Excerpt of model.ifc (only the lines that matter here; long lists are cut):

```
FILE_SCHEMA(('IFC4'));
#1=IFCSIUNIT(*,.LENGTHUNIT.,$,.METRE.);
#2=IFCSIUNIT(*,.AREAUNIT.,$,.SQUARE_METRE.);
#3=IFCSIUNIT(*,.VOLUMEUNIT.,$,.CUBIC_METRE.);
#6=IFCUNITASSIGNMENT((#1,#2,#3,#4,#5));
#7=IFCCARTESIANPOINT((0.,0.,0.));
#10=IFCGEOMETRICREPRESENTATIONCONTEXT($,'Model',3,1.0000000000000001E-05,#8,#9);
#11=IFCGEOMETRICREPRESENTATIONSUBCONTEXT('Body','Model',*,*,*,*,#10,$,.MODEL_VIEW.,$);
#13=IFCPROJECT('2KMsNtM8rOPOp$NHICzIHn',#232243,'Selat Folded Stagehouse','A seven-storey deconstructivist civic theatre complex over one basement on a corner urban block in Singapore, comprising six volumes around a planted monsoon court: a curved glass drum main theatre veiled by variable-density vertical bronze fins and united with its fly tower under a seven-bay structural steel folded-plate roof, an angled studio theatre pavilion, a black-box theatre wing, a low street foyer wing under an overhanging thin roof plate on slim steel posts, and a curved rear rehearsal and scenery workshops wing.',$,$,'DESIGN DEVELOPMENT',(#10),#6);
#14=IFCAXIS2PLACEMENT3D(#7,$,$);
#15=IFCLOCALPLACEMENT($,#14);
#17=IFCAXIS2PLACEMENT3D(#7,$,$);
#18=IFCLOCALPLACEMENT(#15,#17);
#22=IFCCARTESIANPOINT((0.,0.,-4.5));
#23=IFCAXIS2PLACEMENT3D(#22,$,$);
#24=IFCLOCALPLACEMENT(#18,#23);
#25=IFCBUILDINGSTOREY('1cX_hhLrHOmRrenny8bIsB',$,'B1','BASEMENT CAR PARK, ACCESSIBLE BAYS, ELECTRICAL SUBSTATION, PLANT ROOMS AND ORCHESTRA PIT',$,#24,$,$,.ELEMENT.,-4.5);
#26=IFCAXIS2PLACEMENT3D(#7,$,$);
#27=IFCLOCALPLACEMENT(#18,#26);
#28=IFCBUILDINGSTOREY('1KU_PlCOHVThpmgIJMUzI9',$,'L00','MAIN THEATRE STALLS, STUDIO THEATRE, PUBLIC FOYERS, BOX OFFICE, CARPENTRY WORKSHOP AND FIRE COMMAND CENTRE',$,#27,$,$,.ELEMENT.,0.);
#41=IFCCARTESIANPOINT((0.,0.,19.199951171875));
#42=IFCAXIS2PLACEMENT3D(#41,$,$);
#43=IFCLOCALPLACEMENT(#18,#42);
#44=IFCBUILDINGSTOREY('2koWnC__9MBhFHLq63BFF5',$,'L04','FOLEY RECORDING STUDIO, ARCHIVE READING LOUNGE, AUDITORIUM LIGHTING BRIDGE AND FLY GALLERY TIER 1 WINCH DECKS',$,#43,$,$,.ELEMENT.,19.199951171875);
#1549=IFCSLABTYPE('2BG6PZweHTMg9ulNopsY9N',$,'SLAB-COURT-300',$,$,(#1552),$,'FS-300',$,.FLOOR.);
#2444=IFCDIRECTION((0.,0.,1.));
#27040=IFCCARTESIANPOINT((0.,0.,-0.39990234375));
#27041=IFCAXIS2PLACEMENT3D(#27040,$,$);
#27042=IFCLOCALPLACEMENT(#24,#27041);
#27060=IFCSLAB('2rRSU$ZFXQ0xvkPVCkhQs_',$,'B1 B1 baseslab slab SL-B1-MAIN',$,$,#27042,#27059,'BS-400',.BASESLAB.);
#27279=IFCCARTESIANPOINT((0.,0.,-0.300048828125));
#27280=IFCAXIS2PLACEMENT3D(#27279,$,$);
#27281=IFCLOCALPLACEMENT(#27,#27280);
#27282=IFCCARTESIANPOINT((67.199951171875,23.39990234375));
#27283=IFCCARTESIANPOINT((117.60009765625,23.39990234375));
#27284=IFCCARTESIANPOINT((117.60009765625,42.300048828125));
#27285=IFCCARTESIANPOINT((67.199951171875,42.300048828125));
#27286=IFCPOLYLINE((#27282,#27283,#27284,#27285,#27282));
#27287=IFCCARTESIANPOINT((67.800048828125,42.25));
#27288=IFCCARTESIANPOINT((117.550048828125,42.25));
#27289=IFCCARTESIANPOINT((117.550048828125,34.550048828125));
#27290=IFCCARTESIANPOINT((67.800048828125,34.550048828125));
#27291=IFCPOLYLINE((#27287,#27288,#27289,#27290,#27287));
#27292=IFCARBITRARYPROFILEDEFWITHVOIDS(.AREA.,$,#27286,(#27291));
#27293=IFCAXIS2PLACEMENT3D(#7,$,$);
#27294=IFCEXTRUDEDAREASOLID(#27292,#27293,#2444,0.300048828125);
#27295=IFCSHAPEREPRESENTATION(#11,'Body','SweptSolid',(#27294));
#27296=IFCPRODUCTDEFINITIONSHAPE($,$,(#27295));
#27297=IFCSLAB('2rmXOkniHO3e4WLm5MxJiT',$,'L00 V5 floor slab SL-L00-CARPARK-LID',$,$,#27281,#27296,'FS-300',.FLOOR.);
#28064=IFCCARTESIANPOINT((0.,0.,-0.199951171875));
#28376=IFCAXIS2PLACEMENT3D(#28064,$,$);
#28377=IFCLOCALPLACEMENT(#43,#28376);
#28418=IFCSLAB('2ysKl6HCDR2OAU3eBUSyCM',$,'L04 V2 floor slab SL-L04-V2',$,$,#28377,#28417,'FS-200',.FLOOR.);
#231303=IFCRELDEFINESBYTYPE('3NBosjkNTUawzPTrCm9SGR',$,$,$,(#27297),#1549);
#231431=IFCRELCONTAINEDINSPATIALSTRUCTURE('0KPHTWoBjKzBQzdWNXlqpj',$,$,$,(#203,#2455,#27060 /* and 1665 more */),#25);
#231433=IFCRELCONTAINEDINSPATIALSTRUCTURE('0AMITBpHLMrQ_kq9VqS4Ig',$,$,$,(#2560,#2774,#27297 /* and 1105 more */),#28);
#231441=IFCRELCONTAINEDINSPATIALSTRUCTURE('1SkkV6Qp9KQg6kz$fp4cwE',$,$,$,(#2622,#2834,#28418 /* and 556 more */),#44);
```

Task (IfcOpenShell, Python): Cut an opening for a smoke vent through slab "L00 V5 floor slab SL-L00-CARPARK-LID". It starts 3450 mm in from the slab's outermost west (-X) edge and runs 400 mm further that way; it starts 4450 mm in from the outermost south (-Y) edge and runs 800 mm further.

```python
import numpy as np
import ifcopenshell
import ifcopenshell.api.feature
import ifcopenshell.api.geometry
import ifcopenshell.api.root
import ifcopenshell.geom
import ifcopenshell.util.placement
import ifcopenshell.util.representation
import ifcopenshell.util.shape
import ifcopenshell.util.unit

model = ifcopenshell.open("model.ifc")
unit_scale = ifcopenshell.util.unit.calculate_unit_scale(model)
settings = ifcopenshell.geom.settings()


def volume(element):
    """Net volume in cubic metres, openings subtracted."""
    shape = ifcopenshell.geom.create_shape(settings, element)
    return ifcopenshell.util.shape.get_volume(shape.geometry)


slab = model.by_guid("2rmXOkniHO3e4WLm5MxJiT")
before = volume(slab)

# Extent in the slab's own axes, in metres. The edges named are its -X and -Y sides.
slab_shape = ifcopenshell.geom.create_shape(settings, slab)
vertices = ifcopenshell.util.shape.get_vertices(slab_shape.geometry)
x_min, y_min, bottom = vertices.min(axis=0)
top = vertices[:, 2].max()

opening = ifcopenshell.api.root.create_entity(model, ifc_class="IfcOpeningElement", name="Smoke vent opening", predefined_type="OPENING")
context = ifcopenshell.util.representation.get_context(model, "Model", "Body", "MODEL_VIEW")
width, depth = 0.4, 0.8
outline = [(0.0, 0.0), (width, 0.0), (width, depth), (0.0, depth), (0.0, 0.0)]
# Overshoot both faces by 50 mm so the cut is clean.
shape = ifcopenshell.api.geometry.add_slab_representation(
    model, context=context, depth=top - bottom + 0.1, polyline=outline
)
ifcopenshell.api.geometry.assign_representation(model, product=opening, representation=shape)

matrix = ifcopenshell.util.placement.get_local_placement(slab.ObjectPlacement)
matrix[:, 3] = matrix @ np.append(np.array([x_min + 3.45, y_min + 4.45, bottom - 0.05]) / unit_scale, 1.0)
ifcopenshell.api.geometry.edit_object_placement(model, product=opening, matrix=matrix, is_si=False)
ifcopenshell.api.feature.add_feature(model, feature=opening, element=slab)

after = volume(slab)

print(f"slab volume {before:.3f} -> {after:.3f} m3")

model.write("model_v2.ifc")
```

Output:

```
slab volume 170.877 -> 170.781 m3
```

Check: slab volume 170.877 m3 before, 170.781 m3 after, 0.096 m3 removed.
